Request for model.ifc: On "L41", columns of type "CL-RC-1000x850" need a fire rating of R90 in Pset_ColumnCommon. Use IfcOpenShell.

First a look at what the model holds.

```python
import ifcopenshell
import ifcopenshell.util.element

model = ifcopenshell.open("model.ifc")
print(model.schema)
storey = next(s for s in model.by_type("IfcBuildingStorey") if s.Name == "L41")
columns = [e for e in ifcopenshell.util.element.get_decomposition(storey) if e.is_a("IfcColumn")]
seen = {}
for e in columns:
    element_type = ifcopenshell.util.element.get_type(e)
    key = (element_type.Name if element_type != e and element_type else None, ifcopenshell.util.element.get_pset(e, "Pset_ColumnCommon", "FireRating"))
    seen[key] = seen.get(key, 0) + 1
for (name, value), count in sorted(seen.items(), key=str):
    print(count, "x", name, "|", value)
```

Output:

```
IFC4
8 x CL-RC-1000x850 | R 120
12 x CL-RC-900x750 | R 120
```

```python
import ifcopenshell
import ifcopenshell.api.pset
import ifcopenshell.util.element

model = ifcopenshell.open("model.ifc")

storey = next(s for s in model.by_type("IfcBuildingStorey") if s.Name == "L41")
columns = [e for e in ifcopenshell.util.element.get_decomposition(storey) if e.is_a("IfcColumn")]

count = 0
for e in columns:
    element_type = ifcopenshell.util.element.get_type(e)
    if element_type in (None, e) or element_type.Name != "CL-RC-1000x850":
        continue
    found = ifcopenshell.util.element.get_pset(e, "Pset_ColumnCommon", should_inherit=False)
    if found:
        pset = model.by_id(found["id"])
        if len(ifcopenshell.util.element.get_elements_by_pset(pset)) > 1:
            pset = ifcopenshell.api.pset.unshare_pset(model, products=[e], pset=pset)[0]
    else:
        pset = ifcopenshell.api.pset.add_pset(model, product=e, name="Pset_ColumnCommon")
    ifcopenshell.api.pset.edit_pset(model, pset=pset, properties={"FireRating": "R90"})
    count += 1

print(count, "columns updated")

model.write("model-out.ifc")
```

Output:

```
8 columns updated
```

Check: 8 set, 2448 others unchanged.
